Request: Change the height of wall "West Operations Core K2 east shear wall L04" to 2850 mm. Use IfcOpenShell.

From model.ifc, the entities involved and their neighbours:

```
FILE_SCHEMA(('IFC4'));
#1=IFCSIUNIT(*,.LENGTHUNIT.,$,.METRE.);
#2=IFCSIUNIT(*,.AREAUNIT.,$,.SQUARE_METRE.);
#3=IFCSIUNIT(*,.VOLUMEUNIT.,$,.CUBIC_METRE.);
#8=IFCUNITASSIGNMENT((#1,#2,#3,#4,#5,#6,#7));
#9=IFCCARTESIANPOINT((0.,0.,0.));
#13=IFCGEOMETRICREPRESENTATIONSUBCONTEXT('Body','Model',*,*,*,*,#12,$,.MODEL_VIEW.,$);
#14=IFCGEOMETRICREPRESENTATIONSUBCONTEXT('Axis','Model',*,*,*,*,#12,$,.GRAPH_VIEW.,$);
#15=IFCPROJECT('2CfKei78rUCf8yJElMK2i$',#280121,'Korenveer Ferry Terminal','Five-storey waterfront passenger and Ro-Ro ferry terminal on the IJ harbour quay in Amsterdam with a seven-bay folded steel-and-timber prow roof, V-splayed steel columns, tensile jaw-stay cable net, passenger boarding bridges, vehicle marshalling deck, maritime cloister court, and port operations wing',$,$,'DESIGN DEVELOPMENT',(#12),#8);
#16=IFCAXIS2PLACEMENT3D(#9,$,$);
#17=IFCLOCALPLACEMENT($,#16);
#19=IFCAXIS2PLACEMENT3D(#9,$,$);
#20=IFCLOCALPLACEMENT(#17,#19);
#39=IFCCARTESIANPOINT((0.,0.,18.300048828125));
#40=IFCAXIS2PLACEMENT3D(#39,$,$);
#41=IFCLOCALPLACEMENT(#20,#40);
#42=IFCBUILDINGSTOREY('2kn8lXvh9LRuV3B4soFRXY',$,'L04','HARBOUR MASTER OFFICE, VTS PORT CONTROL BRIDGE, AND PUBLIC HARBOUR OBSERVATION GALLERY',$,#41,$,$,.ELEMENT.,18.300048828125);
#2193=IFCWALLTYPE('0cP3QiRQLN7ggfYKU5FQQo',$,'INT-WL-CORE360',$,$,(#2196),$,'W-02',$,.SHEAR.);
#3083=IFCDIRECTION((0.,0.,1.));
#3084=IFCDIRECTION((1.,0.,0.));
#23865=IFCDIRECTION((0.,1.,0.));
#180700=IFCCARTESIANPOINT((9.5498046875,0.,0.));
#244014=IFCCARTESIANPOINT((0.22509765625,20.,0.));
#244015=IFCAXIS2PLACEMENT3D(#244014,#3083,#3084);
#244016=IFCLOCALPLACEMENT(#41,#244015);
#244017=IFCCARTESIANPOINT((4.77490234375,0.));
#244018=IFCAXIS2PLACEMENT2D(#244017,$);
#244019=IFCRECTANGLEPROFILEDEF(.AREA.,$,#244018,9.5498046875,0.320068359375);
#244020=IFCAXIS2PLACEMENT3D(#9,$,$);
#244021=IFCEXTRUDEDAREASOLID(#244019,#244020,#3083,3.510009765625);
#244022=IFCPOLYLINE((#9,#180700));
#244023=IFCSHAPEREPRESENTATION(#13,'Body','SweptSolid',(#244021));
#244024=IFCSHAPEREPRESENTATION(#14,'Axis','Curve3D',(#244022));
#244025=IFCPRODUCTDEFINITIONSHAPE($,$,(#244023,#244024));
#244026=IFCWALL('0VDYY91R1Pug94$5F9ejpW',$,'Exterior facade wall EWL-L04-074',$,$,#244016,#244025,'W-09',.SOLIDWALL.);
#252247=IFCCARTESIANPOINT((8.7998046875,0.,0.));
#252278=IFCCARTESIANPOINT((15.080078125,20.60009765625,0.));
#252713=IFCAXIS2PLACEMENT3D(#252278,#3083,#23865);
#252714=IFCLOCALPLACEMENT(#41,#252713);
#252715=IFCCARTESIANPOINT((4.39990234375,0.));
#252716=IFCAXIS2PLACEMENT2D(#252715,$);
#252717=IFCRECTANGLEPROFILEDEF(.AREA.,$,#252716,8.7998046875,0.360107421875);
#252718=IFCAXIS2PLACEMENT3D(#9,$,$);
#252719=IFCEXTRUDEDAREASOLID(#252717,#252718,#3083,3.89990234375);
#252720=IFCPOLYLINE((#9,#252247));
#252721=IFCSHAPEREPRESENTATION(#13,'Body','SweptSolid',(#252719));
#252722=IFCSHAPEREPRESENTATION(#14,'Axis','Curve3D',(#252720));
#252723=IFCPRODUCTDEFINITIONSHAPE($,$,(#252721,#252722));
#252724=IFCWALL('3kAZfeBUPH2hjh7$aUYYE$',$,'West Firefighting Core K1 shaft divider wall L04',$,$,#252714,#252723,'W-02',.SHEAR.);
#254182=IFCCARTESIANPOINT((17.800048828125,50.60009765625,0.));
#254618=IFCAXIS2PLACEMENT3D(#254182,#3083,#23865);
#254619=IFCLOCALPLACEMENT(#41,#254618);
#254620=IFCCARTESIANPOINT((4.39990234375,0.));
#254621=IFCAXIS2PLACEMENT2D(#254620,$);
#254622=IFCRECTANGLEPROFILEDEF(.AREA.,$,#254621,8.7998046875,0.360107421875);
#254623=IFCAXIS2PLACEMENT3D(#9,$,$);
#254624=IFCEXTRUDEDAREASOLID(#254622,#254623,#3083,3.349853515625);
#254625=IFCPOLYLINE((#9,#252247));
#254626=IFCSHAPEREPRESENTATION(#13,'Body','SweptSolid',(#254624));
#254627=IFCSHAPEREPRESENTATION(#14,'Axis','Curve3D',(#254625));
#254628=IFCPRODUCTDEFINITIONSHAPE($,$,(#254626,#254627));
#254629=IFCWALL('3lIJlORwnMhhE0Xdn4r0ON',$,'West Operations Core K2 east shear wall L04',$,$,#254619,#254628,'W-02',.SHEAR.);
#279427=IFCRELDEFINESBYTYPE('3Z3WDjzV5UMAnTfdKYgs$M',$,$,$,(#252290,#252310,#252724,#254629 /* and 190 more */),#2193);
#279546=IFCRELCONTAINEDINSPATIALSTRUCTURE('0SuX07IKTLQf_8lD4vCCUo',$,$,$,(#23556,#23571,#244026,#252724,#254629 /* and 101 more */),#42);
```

```python
import ifcopenshell
import ifcopenshell.geom
import ifcopenshell.util.representation
import ifcopenshell.util.shape
import ifcopenshell.util.unit

model = ifcopenshell.open("model.ifc")
unit_scale = ifcopenshell.util.unit.calculate_unit_scale(model)
settings = ifcopenshell.geom.settings()


def volume(element):
    """Net volume in cubic metres, openings subtracted."""
    shape = ifcopenshell.geom.create_shape(settings, element)
    return ifcopenshell.util.shape.get_volume(shape.geometry)


wall = model.by_guid("3lIJlORwnMhhE0Xdn4r0ON")
before = volume(wall)

body = ifcopenshell.util.representation.get_representation(wall, "Model", "Body")
solid = body.Items[0]
old_height = solid.Depth
solid.Depth = 2.85 / unit_scale
after = volume(wall)

print(f"height {old_height:g} -> {solid.Depth:g}, volume {before:.3f} -> {after:.3f} m3")

model.write("model_updated.ifc")
```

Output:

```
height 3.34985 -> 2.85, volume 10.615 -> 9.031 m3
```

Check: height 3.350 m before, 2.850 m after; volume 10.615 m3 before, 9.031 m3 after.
